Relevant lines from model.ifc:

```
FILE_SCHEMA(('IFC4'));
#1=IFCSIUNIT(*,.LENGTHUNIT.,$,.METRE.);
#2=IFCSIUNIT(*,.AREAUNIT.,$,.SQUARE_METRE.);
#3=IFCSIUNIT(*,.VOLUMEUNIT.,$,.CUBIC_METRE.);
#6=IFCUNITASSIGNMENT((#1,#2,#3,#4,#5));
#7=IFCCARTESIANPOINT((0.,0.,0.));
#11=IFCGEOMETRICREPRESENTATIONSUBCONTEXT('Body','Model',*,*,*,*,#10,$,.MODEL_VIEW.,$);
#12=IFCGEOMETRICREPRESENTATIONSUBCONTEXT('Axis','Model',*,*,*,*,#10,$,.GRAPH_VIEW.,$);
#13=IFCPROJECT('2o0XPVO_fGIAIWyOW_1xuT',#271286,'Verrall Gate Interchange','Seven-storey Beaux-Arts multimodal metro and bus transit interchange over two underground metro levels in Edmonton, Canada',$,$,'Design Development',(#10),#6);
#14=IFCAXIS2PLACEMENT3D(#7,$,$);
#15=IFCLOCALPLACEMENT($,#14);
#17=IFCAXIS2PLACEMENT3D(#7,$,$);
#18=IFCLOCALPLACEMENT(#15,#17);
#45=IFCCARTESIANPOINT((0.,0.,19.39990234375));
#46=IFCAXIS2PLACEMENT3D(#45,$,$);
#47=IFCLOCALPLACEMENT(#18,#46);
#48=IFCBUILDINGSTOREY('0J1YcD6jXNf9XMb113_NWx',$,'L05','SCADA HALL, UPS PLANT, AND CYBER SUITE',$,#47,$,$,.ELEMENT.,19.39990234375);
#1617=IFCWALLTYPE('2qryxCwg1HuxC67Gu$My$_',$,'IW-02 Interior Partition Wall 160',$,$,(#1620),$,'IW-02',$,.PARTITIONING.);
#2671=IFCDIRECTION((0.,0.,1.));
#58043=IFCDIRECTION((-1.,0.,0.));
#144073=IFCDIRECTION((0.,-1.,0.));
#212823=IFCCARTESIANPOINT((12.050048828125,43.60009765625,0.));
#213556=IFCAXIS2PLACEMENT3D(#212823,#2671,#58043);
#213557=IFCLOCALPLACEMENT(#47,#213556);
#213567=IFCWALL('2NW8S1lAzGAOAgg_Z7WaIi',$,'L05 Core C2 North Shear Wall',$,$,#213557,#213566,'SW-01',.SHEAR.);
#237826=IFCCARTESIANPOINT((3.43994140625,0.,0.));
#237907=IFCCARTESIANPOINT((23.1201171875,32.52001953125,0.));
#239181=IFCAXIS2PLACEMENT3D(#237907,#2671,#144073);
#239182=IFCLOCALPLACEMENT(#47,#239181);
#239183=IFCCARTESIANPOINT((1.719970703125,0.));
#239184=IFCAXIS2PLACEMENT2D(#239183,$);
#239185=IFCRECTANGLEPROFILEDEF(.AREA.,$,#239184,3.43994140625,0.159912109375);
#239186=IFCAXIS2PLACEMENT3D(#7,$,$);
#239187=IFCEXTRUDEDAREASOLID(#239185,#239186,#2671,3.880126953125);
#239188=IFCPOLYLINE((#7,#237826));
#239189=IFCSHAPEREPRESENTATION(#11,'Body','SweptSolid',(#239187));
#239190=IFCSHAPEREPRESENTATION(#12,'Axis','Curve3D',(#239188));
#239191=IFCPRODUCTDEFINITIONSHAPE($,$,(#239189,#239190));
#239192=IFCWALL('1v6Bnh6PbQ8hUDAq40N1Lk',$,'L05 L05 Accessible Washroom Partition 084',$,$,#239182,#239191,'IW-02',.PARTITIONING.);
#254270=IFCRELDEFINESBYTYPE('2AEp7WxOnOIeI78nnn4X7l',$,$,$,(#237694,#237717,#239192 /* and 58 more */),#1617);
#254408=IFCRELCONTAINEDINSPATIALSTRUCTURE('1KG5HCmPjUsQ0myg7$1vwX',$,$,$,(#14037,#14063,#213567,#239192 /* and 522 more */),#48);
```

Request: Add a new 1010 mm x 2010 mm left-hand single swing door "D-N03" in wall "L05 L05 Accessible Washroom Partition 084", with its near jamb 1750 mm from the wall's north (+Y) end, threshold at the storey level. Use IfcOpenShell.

```python
import numpy as np
import ifcopenshell
import ifcopenshell.api.feature
import ifcopenshell.api.geometry
import ifcopenshell.api.root
import ifcopenshell.api.spatial
import ifcopenshell.geom
import ifcopenshell.util.element
import ifcopenshell.util.placement
import ifcopenshell.util.representation
import ifcopenshell.util.shape
import ifcopenshell.util.unit

model = ifcopenshell.open("model.ifc")
unit_scale = ifcopenshell.util.unit.calculate_unit_scale(model)
settings = ifcopenshell.geom.settings()


def volume(element):
    """Net volume in cubic metres, openings subtracted."""
    shape = ifcopenshell.geom.create_shape(settings, element)
    return ifcopenshell.util.shape.get_volume(shape.geometry)


wall = model.by_guid("1v6Bnh6PbQ8hUDAq40N1Lk")
storey = ifcopenshell.util.element.get_container(wall, ifc_class="IfcBuildingStorey")
context = ifcopenshell.util.representation.get_context(model, "Model", "Body", "MODEL_VIEW")
before = volume(wall)

width, height, from_end, sill = 1.01, 2.01, 1.75, 0.0  # metres

# The wall runs along its own X axis, and the end named is its -X end.
wall_shape = ifcopenshell.geom.create_shape(settings, wall)
x, y, z = ifcopenshell.util.shape.get_vertices(wall_shape.geometry).T
start = x.min() + from_end
face, thickness = float(y.min()), float(y.max() - y.min())
wall_matrix = ifcopenshell.util.placement.get_local_placement(wall.ObjectPlacement)
level = ifcopenshell.util.placement.get_local_placement(storey.ObjectPlacement)[2, 3]


def in_wall(x, y):
    """Placement at x, y metres in the wall's axes, at sill height."""
    matrix = wall_matrix.copy()
    matrix[:, 3] = wall_matrix @ np.array([x / unit_scale, y / unit_scale, 0.0, 1.0])
    matrix[2, 3] = level + sill / unit_scale
    return matrix


# Opening: a box that overshoots both wall faces by 50 mm.
opening = ifcopenshell.api.root.create_entity(model, ifc_class="IfcOpeningElement", predefined_type="OPENING")
box = ifcopenshell.api.geometry.add_wall_representation(
    model, context=context, length=width, height=height, thickness=thickness + 0.1
)
ifcopenshell.api.geometry.assign_representation(model, product=opening, representation=box)
ifcopenshell.api.geometry.edit_object_placement(model, product=opening, matrix=in_wall(start, face - 0.05), is_si=False)
ifcopenshell.api.feature.add_feature(model, feature=opening, element=wall)

door = ifcopenshell.api.root.create_entity(model, ifc_class="IfcDoor", name="D-N03", predefined_type="DOOR")
door.OverallWidth, door.OverallHeight = width / unit_scale, height / unit_scale
door.OperationType = "SINGLE_SWING_LEFT"
body = ifcopenshell.api.geometry.add_door_representation(
    model,
    context=context,
    overall_width=door.OverallWidth,
    overall_height=door.OverallHeight,
    operation_type="SINGLE_SWING_LEFT",
    lining_properties={"LiningDepth": thickness / unit_scale, "ThresholdDepth": thickness / unit_scale},
)
ifcopenshell.api.geometry.assign_representation(model, product=door, representation=body)
ifcopenshell.api.spatial.assign_container(model, products=[door], relating_structure=storey)
ifcopenshell.api.feature.add_filling(model, opening=opening, element=door)

# The lining spans the wall, so the door starts at the wall face.
ifcopenshell.api.geometry.edit_object_placement(model, product=door, matrix=in_wall(start, face), is_si=False)

after = volume(wall)

print(f"wall volume {before:.3f} -> {after:.3f} m3")

model.write("model-out.ifc")
```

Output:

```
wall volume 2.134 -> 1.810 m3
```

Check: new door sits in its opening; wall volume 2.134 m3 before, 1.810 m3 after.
